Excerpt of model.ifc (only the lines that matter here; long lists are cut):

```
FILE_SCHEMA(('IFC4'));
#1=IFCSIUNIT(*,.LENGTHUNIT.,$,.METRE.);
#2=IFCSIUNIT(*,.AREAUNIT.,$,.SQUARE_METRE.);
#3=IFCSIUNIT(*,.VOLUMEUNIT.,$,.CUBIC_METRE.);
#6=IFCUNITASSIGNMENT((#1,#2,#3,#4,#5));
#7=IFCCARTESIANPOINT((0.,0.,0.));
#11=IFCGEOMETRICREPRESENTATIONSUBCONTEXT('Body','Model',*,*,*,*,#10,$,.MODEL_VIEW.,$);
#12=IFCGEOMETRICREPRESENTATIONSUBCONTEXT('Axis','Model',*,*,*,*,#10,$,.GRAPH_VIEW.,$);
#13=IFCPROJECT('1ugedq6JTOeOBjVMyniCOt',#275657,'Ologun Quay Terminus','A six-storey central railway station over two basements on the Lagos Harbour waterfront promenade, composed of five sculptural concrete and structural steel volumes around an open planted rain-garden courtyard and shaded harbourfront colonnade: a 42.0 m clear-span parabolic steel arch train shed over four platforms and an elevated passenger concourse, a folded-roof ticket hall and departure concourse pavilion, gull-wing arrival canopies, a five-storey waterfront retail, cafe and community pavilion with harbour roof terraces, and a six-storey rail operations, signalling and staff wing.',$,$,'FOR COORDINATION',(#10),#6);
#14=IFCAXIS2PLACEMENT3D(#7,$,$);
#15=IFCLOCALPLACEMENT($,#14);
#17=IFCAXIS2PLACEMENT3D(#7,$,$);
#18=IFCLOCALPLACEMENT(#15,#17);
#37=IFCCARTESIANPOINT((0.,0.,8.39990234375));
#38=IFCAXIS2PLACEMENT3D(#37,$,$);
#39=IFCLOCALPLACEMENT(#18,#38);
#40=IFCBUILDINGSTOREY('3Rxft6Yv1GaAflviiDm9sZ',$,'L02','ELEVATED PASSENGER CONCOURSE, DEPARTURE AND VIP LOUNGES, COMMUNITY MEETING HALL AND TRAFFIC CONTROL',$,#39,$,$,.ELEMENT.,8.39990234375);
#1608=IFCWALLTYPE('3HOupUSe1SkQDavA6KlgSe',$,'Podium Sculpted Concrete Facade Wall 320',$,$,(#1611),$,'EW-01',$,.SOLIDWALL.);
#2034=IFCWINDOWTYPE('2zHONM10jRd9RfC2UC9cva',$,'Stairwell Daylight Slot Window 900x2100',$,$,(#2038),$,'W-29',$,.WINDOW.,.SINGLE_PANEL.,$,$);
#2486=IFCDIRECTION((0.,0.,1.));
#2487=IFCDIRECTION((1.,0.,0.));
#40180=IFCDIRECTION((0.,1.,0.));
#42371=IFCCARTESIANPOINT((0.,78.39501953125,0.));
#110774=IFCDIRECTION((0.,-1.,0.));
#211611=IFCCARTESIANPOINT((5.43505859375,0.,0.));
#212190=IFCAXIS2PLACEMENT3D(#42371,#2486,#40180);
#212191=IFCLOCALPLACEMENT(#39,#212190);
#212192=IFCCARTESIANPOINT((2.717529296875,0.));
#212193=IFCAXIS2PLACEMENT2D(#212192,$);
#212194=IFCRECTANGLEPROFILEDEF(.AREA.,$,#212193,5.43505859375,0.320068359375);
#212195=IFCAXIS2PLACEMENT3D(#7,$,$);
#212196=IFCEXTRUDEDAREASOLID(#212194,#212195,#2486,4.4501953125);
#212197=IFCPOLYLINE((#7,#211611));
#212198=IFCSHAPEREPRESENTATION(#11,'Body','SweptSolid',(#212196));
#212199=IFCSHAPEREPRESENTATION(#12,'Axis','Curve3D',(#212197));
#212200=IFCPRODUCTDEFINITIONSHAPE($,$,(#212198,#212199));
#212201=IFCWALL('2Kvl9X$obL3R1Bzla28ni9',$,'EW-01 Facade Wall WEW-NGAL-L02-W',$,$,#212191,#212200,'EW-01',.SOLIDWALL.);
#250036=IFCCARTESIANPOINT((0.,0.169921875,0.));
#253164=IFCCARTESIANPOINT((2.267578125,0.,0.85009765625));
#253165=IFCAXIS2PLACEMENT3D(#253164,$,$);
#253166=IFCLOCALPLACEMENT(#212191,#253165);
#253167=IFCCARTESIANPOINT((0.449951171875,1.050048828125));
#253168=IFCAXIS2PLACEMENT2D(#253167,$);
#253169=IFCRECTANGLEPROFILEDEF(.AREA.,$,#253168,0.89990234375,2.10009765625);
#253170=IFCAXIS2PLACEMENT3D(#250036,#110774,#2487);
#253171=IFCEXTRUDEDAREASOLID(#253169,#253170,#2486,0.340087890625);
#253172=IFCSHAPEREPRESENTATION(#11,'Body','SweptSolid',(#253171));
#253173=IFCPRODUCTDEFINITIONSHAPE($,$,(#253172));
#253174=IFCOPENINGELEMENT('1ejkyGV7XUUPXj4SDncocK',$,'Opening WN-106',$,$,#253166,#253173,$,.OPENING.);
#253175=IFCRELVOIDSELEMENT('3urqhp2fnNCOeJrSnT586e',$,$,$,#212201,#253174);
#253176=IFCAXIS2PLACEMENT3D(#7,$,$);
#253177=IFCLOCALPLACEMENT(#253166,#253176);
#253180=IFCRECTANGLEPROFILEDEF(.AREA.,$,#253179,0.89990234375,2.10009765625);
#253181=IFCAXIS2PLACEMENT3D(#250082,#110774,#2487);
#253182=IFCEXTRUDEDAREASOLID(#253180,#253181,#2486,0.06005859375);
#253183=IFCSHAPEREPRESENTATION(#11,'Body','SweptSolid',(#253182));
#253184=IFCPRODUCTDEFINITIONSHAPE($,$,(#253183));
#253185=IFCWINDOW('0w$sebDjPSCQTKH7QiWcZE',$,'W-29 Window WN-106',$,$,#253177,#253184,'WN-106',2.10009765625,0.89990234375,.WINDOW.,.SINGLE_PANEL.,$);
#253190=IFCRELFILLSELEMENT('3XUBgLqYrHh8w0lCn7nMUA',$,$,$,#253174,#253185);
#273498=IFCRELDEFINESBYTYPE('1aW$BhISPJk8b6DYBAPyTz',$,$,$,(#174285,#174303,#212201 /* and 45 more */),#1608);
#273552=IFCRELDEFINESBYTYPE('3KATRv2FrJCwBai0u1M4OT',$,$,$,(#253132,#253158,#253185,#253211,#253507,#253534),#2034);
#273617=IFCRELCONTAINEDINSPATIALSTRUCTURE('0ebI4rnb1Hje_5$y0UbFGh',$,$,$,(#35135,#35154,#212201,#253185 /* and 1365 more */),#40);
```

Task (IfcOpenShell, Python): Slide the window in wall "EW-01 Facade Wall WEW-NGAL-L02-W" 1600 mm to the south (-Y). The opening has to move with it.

```python
import ifcopenshell
import ifcopenshell.api.geometry
import ifcopenshell.util.placement
import ifcopenshell.util.unit

model = ifcopenshell.open("model.ifc")
unit_scale = ifcopenshell.util.unit.calculate_unit_scale(model)

window = model.by_guid("0w$sebDjPSCQTKH7QiWcZE")
opening = window.FillsVoids[0].RelatingOpeningElement
wall = opening.VoidsElements[0].RelatingBuildingElement

wall_matrix = ifcopenshell.util.placement.get_local_placement(wall.ObjectPlacement)
shift = wall_matrix[:3, 0] * -1.6 / unit_scale
before = ifcopenshell.util.placement.get_local_placement(window.ObjectPlacement)[:3, 3].copy()

# The window is placed relative to its opening, so it follows when the opening moves.
matrix = ifcopenshell.util.placement.get_local_placement(opening.ObjectPlacement)
matrix[:3, 3] += shift
ifcopenshell.api.geometry.edit_object_placement(
    model, product=opening, matrix=matrix, is_si=False, should_transform_children=True
)

after = ifcopenshell.util.placement.get_local_placement(window.ObjectPlacement)[:3, 3]
print("window moved by", (after - before).round(3) + 0.0)

model.write("model-out.ifc")
```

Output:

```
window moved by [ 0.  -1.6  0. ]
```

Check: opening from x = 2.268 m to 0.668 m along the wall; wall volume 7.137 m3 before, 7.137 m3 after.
